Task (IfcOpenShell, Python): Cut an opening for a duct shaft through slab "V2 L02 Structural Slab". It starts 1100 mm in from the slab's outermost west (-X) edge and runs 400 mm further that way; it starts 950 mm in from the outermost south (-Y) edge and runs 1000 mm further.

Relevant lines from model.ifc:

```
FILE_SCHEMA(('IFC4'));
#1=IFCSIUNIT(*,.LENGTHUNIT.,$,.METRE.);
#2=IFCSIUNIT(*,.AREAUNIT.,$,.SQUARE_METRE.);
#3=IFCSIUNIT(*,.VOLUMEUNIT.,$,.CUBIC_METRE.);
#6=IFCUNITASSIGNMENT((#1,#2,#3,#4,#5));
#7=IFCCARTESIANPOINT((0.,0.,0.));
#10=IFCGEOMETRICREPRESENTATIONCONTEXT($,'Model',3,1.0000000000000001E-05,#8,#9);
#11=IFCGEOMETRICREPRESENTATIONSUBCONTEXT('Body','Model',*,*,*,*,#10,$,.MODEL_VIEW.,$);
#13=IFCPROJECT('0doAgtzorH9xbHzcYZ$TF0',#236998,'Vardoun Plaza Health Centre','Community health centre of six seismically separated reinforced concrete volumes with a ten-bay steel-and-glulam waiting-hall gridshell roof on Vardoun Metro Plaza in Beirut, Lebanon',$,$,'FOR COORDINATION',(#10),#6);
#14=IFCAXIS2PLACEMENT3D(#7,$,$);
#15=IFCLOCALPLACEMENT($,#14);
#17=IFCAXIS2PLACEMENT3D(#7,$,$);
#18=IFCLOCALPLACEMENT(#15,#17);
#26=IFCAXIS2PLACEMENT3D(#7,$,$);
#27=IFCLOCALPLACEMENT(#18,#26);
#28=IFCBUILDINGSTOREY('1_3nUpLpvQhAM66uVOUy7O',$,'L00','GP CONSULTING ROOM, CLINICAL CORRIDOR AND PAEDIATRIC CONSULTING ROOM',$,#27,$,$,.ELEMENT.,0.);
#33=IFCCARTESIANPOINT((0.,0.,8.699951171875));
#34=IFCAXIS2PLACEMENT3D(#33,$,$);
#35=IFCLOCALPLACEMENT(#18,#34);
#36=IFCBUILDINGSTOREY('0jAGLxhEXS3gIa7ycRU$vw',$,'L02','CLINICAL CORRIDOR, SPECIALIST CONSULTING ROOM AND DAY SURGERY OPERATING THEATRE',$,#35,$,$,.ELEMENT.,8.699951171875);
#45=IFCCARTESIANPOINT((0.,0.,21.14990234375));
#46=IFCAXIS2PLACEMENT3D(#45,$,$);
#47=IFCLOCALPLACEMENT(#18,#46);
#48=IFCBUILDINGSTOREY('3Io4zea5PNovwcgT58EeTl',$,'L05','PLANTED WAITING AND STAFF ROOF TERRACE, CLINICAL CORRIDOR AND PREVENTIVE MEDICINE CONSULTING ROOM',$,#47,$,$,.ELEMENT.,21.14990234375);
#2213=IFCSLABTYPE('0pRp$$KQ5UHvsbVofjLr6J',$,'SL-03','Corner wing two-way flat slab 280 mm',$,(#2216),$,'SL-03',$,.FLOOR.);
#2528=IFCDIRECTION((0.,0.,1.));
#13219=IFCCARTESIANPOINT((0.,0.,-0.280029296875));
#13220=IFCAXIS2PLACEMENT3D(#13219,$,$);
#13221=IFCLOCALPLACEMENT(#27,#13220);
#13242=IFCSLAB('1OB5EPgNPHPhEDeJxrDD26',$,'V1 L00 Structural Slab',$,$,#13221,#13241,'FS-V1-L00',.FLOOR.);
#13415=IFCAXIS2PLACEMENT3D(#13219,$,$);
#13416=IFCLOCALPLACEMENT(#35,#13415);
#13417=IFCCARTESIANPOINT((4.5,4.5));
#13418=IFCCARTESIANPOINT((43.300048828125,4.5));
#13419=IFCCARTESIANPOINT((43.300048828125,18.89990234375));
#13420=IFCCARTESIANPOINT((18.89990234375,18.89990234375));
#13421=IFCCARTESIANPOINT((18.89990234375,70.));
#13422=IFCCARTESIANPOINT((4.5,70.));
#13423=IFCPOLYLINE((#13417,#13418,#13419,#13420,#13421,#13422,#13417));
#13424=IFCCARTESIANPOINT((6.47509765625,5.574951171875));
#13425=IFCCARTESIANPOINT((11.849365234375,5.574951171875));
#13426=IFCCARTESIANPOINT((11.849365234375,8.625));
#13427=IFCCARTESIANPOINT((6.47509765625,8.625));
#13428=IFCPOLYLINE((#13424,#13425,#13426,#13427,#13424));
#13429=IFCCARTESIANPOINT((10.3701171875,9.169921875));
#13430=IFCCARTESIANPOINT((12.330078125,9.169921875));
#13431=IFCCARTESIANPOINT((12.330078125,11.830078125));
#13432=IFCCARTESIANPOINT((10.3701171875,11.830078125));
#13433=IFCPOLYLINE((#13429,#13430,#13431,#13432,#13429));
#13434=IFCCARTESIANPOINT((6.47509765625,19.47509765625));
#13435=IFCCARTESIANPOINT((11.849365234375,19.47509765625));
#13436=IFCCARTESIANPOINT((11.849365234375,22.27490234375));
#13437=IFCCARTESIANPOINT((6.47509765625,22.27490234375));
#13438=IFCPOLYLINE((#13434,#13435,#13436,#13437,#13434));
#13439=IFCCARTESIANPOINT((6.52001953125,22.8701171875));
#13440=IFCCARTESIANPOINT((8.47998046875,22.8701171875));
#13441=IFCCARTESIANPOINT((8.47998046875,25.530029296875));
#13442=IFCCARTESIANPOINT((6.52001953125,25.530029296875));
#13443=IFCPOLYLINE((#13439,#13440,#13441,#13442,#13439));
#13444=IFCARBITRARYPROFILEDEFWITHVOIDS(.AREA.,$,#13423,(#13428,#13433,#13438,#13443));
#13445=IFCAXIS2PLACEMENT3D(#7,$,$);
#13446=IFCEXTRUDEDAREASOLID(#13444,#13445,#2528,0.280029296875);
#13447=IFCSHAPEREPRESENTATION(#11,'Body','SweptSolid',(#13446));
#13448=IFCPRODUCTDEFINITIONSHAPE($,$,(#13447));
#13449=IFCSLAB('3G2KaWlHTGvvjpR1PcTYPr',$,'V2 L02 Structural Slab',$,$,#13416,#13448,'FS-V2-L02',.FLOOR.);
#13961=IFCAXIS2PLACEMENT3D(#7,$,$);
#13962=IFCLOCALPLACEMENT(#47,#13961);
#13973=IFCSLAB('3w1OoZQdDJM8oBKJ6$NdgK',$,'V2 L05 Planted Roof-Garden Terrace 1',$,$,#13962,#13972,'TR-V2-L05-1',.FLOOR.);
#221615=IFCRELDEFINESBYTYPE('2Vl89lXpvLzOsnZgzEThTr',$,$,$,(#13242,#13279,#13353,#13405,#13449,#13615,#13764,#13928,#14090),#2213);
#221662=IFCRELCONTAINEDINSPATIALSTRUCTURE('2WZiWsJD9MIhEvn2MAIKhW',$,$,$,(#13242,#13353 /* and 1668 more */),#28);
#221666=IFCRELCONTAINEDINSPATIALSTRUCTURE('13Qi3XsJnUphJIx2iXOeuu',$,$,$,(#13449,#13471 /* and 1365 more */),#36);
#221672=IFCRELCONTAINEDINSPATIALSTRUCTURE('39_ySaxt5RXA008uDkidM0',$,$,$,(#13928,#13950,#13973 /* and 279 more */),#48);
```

```python
import numpy as np
import ifcopenshell
import ifcopenshell.api.feature
import ifcopenshell.api.geometry
import ifcopenshell.api.root
import ifcopenshell.geom
import ifcopenshell.util.placement
import ifcopenshell.util.representation
import ifcopenshell.util.shape
import ifcopenshell.util.unit

model = ifcopenshell.open("model.ifc")
unit_scale = ifcopenshell.util.unit.calculate_unit_scale(model)
settings = ifcopenshell.geom.settings()


def volume(element):
    """Net volume in cubic metres, openings subtracted."""
    shape = ifcopenshell.geom.create_shape(settings, element)
    return ifcopenshell.util.shape.get_volume(shape.geometry)


slab = model.by_id(13449)
before = volume(slab)

# Extent in the slab's own axes, in metres. The edges named are its -X and -Y sides.
slab_shape = ifcopenshell.geom.create_shape(settings, slab)
vertices = ifcopenshell.util.shape.get_vertices(slab_shape.geometry)
x_min, y_min, bottom = vertices.min(axis=0)
top = vertices[:, 2].max()

opening = ifcopenshell.api.root.create_entity(model, ifc_class="IfcOpeningElement", name="Duct shaft opening", predefined_type="OPENING")
context = ifcopenshell.util.representation.get_context(model, "Model", "Body", "MODEL_VIEW")
width, depth = 0.4, 1
outline = [(0.0, 0.0), (width, 0.0), (width, depth), (0.0, depth), (0.0, 0.0)]
# Overshoot both faces by 50 mm so the cut is clean.
shape = ifcopenshell.api.geometry.add_slab_representation(
    model, context=context, depth=top - bottom + 0.1, polyline=outline
)
ifcopenshell.api.geometry.assign_representation(model, product=opening, representation=shape)

matrix = ifcopenshell.util.placement.get_local_placement(slab.ObjectPlacement)
matrix[:, 3] = matrix @ np.append(np.array([x_min + 1.1, y_min + 0.95, bottom - 0.05]) / unit_scale, 1.0)
ifcopenshell.api.geometry.edit_object_placement(model, product=opening, matrix=matrix, is_si=False)
ifcopenshell.api.feature.add_feature(model, feature=opening, element=slab)

after = volume(slab)

print(f"slab volume {before:.3f} -> {after:.3f} m3")

model.write("model_edited.ifc")
```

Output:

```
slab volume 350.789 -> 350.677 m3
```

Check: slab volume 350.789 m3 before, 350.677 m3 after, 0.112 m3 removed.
